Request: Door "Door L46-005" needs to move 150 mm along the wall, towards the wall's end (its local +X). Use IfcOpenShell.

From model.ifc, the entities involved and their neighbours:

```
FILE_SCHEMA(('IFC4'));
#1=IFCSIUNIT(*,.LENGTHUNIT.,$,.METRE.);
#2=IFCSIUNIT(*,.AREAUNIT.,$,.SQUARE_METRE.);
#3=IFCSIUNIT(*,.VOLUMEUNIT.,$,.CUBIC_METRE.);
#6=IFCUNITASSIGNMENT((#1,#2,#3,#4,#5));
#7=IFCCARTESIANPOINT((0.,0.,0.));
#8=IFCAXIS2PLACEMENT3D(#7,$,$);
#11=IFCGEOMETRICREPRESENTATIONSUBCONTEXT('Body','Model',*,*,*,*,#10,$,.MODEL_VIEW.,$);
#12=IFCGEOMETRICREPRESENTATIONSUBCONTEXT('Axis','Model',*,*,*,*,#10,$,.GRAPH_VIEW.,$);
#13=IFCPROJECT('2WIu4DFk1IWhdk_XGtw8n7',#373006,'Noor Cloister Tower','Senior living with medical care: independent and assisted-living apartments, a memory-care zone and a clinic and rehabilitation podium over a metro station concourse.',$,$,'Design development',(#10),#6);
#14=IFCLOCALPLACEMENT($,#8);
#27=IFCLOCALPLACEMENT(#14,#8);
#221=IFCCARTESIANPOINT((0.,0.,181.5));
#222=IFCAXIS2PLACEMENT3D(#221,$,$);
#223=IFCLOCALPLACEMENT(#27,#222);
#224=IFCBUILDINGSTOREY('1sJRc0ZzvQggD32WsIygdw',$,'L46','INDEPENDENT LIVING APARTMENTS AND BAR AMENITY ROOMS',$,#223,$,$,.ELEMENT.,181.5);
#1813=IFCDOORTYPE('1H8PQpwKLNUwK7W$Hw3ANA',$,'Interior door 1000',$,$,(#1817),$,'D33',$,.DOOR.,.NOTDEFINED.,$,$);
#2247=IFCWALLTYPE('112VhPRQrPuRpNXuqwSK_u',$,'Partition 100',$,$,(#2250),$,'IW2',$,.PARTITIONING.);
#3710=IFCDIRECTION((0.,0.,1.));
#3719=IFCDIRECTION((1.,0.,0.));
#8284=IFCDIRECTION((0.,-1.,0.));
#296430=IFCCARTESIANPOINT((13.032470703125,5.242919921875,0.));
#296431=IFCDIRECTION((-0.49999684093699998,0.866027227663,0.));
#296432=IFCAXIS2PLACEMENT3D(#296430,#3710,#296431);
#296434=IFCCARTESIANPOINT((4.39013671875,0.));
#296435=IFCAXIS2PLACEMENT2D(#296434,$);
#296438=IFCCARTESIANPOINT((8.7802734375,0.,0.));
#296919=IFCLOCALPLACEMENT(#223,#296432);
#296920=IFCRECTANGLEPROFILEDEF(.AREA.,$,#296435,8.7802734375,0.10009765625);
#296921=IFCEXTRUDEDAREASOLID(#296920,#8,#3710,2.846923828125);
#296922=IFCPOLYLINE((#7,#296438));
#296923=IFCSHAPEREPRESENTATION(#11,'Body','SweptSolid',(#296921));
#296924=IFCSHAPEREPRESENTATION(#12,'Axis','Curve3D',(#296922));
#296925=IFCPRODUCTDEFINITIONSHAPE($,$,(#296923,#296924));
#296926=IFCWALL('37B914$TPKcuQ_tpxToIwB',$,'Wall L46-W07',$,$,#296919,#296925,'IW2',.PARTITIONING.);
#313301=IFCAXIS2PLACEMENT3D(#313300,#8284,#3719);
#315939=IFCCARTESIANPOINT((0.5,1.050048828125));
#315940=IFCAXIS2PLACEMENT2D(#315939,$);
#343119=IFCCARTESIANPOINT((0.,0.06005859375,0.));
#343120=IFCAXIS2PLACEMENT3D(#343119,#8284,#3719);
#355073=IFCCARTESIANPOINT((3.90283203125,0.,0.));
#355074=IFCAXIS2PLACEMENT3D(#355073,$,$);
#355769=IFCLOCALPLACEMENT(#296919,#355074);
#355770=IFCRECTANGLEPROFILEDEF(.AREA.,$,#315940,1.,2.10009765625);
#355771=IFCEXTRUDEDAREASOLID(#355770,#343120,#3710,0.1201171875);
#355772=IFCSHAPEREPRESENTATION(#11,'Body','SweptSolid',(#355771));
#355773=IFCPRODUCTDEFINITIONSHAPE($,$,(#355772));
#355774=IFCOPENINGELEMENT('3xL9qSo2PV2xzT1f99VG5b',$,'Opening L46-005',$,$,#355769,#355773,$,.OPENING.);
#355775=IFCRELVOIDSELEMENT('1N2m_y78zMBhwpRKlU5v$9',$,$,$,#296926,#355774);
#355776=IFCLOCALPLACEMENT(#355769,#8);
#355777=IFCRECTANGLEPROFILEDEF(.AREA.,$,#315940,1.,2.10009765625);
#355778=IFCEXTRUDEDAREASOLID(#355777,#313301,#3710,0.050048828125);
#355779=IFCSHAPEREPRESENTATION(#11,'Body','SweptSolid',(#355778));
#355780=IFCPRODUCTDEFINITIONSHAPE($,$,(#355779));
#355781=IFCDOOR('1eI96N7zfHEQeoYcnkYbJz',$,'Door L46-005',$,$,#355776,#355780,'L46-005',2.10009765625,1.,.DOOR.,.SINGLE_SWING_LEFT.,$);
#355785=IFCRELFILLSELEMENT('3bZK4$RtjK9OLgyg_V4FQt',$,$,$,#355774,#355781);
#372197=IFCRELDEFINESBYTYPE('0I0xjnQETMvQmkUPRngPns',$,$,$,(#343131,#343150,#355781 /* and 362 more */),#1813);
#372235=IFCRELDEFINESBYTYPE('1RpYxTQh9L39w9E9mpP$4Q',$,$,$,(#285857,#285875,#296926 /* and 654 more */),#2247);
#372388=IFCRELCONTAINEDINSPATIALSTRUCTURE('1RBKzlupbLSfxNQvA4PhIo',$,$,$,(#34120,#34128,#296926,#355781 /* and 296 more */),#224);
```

```python
import ifcopenshell
import ifcopenshell.api.geometry
import ifcopenshell.util.placement

model = ifcopenshell.open("model.ifc")

door = model.by_id(355781)
opening = door.FillsVoids[0].RelatingOpeningElement
wall = opening.VoidsElements[0].RelatingBuildingElement

wall_matrix = ifcopenshell.util.placement.get_local_placement(wall.ObjectPlacement)
shift = wall_matrix[:3, 0] * 0.15
before = ifcopenshell.util.placement.get_local_placement(door.ObjectPlacement)[:3, 3].copy()

# The door is placed relative to its opening, so it follows when the opening moves.
matrix = ifcopenshell.util.placement.get_local_placement(opening.ObjectPlacement)
matrix[:3, 3] += shift
ifcopenshell.api.geometry.edit_object_placement(
    model, product=opening, matrix=matrix, is_si=False, should_transform_children=True
)

after = ifcopenshell.util.placement.get_local_placement(door.ObjectPlacement)[:3, 3]
print("door moved by", (after - before).round(3) + 0.0)

model.write("model_updated.ifc")
```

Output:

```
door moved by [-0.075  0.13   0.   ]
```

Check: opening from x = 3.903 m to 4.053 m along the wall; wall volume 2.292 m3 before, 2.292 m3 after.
